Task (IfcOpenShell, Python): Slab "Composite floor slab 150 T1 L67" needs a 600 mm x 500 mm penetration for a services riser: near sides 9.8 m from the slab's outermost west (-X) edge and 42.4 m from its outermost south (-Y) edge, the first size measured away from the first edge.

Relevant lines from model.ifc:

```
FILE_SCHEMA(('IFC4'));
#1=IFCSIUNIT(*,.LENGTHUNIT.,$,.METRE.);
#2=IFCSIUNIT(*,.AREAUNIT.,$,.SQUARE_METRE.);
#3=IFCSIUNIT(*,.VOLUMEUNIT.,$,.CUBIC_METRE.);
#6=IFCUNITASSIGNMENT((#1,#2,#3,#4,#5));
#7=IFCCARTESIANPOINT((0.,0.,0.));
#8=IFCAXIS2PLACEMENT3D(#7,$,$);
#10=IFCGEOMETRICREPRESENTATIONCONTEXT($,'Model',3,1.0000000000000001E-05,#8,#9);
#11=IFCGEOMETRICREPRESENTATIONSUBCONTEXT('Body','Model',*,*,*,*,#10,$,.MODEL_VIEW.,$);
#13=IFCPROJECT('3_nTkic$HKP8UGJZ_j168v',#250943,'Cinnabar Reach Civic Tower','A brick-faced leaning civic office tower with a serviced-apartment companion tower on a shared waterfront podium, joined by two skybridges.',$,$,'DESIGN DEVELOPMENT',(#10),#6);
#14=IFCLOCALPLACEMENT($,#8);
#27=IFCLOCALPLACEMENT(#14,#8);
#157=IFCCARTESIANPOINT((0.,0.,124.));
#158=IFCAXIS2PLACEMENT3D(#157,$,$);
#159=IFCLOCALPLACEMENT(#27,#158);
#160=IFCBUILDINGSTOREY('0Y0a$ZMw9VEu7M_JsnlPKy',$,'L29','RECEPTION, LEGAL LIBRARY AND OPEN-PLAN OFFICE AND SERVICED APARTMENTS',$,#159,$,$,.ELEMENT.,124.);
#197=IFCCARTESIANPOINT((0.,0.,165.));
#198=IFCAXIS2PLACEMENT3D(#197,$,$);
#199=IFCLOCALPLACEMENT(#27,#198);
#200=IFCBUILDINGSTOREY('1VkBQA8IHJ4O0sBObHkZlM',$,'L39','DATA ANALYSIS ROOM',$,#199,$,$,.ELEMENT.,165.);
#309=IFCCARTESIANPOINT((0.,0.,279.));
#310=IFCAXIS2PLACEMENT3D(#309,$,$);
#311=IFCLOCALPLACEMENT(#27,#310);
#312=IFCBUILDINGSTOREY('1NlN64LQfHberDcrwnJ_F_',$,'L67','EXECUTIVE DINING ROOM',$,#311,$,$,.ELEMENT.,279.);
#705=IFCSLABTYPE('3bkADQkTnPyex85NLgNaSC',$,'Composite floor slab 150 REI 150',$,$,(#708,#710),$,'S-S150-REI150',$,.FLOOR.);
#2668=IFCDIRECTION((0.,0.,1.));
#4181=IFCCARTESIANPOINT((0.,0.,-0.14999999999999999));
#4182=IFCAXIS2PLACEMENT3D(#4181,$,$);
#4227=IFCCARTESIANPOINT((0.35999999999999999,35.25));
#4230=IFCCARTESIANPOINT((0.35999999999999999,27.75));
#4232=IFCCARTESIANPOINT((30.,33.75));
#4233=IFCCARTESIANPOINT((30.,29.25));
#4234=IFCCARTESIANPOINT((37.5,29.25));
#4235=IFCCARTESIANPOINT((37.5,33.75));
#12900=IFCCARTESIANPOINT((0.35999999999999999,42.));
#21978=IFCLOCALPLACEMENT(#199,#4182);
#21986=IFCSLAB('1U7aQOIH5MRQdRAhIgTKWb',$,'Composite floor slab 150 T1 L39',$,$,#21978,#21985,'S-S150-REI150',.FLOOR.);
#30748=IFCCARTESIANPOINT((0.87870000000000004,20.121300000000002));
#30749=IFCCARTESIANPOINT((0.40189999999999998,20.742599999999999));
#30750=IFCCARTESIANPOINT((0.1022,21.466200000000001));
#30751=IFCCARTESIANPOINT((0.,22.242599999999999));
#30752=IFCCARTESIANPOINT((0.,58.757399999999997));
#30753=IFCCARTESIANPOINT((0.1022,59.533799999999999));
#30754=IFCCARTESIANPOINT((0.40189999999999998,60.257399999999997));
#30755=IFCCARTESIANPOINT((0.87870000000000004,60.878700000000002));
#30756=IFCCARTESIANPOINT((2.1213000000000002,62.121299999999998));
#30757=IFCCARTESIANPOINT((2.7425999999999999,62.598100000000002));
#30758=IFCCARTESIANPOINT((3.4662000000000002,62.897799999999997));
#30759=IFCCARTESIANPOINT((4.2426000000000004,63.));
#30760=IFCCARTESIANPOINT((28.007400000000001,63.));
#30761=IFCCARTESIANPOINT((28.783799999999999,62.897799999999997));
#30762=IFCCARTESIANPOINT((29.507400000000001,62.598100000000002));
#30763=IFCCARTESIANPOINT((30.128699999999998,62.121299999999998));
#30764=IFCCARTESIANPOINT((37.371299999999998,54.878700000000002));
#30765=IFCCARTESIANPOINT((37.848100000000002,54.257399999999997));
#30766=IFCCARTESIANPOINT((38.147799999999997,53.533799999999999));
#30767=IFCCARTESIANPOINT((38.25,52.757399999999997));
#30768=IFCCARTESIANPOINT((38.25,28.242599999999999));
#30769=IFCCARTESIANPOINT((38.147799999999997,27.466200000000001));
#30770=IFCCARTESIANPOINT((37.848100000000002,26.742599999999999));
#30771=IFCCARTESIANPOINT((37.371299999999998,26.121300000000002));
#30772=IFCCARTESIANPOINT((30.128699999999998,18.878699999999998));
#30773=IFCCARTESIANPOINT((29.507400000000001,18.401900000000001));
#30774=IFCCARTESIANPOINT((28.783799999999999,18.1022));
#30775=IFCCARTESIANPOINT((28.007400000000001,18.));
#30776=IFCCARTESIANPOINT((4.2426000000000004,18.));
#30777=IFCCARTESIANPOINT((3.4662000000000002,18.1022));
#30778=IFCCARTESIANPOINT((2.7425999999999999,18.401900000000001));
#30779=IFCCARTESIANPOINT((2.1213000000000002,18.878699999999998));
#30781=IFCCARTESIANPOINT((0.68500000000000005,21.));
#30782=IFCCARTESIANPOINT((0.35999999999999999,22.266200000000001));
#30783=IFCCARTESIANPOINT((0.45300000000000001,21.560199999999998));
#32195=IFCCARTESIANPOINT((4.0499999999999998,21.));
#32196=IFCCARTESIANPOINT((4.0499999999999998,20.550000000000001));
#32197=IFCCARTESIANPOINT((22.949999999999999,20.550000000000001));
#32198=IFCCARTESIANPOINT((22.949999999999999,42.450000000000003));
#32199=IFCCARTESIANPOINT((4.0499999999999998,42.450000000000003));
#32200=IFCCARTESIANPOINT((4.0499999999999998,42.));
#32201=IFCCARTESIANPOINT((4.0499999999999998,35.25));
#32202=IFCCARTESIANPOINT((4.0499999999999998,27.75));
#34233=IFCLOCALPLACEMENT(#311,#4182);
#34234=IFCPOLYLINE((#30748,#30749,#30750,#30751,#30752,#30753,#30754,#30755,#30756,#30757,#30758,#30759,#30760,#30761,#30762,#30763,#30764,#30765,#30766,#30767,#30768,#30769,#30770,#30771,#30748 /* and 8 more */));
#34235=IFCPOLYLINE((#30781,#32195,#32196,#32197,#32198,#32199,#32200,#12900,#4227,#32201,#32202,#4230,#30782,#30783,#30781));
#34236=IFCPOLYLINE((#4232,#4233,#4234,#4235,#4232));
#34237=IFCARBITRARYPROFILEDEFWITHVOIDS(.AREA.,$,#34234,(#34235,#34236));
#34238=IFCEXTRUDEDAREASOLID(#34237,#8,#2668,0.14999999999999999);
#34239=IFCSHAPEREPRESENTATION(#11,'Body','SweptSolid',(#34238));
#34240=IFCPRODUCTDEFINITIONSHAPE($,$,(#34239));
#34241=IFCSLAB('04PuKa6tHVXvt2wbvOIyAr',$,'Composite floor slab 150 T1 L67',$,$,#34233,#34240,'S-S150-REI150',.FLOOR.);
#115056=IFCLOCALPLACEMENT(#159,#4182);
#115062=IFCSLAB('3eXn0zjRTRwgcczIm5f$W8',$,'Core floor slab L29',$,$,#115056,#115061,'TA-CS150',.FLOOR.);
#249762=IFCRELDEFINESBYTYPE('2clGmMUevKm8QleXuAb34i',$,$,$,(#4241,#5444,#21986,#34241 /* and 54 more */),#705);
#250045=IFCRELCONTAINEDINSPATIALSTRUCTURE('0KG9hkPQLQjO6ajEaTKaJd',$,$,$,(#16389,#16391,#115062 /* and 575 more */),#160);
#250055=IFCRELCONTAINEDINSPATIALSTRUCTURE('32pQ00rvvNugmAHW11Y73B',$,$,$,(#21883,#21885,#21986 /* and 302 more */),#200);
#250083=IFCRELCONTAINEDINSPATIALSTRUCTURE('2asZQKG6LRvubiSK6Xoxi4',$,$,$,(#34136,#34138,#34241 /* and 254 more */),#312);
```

```python
import numpy as np
import ifcopenshell
import ifcopenshell.api.feature
import ifcopenshell.api.geometry
import ifcopenshell.api.root
import ifcopenshell.geom
import ifcopenshell.util.placement
import ifcopenshell.util.representation
import ifcopenshell.util.shape
import ifcopenshell.util.unit

model = ifcopenshell.open("model.ifc")
unit_scale = ifcopenshell.util.unit.calculate_unit_scale(model)
settings = ifcopenshell.geom.settings()


def volume(element):
    """Net volume in cubic metres, openings subtracted."""
    shape = ifcopenshell.geom.create_shape(settings, element)
    return ifcopenshell.util.shape.get_volume(shape.geometry)


slab = model.by_guid("04PuKa6tHVXvt2wbvOIyAr")
before = volume(slab)

# Extent in the slab's own axes, in metres. The edges named are its -X and -Y sides.
slab_shape = ifcopenshell.geom.create_shape(settings, slab)
vertices = ifcopenshell.util.shape.get_vertices(slab_shape.geometry)
x_min, y_min, bottom = vertices.min(axis=0)
top = vertices[:, 2].max()

opening = ifcopenshell.api.root.create_entity(model, ifc_class="IfcOpeningElement", name="Services riser opening", predefined_type="OPENING")
context = ifcopenshell.util.representation.get_context(model, "Model", "Body", "MODEL_VIEW")
width, depth = 0.6, 0.5
outline = [(0.0, 0.0), (width, 0.0), (width, depth), (0.0, depth), (0.0, 0.0)]
# Overshoot both faces by 50 mm so the cut is clean.
shape = ifcopenshell.api.geometry.add_slab_representation(
    model, context=context, depth=top - bottom + 0.1, polyline=outline
)
ifcopenshell.api.geometry.assign_representation(model, product=opening, representation=shape)

matrix = ifcopenshell.util.placement.get_local_placement(slab.ObjectPlacement)
matrix[:, 3] = matrix @ np.append(np.array([x_min + 9.8, y_min + 42.4, bottom - 0.05]) / unit_scale, 1.0)
ifcopenshell.api.geometry.edit_object_placement(model, product=opening, matrix=matrix, is_si=False)
ifcopenshell.api.feature.add_feature(model, feature=opening, element=slab)

after = volume(slab)

print(f"slab volume {before:.3f} -> {after:.3f} m3")

model.write("model-out.ifc")
```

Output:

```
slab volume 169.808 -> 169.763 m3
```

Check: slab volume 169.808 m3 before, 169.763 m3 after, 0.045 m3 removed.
